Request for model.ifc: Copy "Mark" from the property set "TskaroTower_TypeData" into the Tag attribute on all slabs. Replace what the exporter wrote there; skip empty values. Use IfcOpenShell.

First a look at what the model holds.

```python
import ifcopenshell
import ifcopenshell.util.element

model = ifcopenshell.open("model.ifc")
print(model.schema)
slabs = model.by_type("IfcSlab")
print(len(slabs), "slabs")
for e in slabs[:8]:
    source = ifcopenshell.util.element.get_pset(e, "TskaroTower_TypeData", "Mark")
    target = e.Tag
    print(e.id(), repr(source), repr(target), sep=" | ")
```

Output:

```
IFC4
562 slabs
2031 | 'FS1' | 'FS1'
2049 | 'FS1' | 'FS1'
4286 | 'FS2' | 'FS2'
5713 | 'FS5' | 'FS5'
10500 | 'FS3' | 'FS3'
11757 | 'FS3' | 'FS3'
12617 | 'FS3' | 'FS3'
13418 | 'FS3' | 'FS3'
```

```python
import ifcopenshell
import ifcopenshell.util.element

model = ifcopenshell.open("model.ifc")

count = 0
for e in model.by_type("IfcSlab"):
    value = ifcopenshell.util.element.get_pset(e, "TskaroTower_TypeData", "Mark")
    current = e.Tag
    if not value or not value.strip() or current == value:
        continue
    e.Tag = value
    count += 1

print(count, "slabs updated")

model.write("model_rev.ifc")
```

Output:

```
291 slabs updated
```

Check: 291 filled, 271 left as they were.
